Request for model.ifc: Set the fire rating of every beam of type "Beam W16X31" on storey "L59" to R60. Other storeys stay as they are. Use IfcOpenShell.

First a look at what the model holds.

```python
import ifcopenshell
import ifcopenshell.util.element

model = ifcopenshell.open("model.ifc")
print(model.schema)
storey = next(s for s in model.by_type("IfcBuildingStorey") if s.Name == "L59")
beams = [e for e in ifcopenshell.util.element.get_decomposition(storey) if e.is_a("IfcBeam")]
seen = {}
for e in beams:
    element_type = ifcopenshell.util.element.get_type(e)
    key = (element_type.Name if element_type != e and element_type else None, ifcopenshell.util.element.get_pset(e, "Pset_BeamCommon", "FireRating"))
    seen[key] = seen.get(key, 0) + 1
for (name, value), count in sorted(seen.items(), key=str):
    print(count, "x", name, "|", value)
```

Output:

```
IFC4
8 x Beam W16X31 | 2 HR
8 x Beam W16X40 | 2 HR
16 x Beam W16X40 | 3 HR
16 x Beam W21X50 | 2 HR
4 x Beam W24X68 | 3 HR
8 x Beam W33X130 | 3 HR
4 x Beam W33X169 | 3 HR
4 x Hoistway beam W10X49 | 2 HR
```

```python
import ifcopenshell
import ifcopenshell.api.pset
import ifcopenshell.util.element

model = ifcopenshell.open("model.ifc")

storey = next(s for s in model.by_type("IfcBuildingStorey") if s.Name == "L59")
beams = [e for e in ifcopenshell.util.element.get_decomposition(storey) if e.is_a("IfcBeam")]

count = 0
for e in beams:
    element_type = ifcopenshell.util.element.get_type(e)
    if element_type in (None, e) or element_type.Name != "Beam W16X31":
        continue
    found = ifcopenshell.util.element.get_pset(e, "Pset_BeamCommon", should_inherit=False)
    if found:
        pset = model.by_id(found["id"])
        if len(ifcopenshell.util.element.get_elements_by_pset(pset)) > 1:
            pset = ifcopenshell.api.pset.unshare_pset(model, products=[e], pset=pset)[0]
    else:
        pset = ifcopenshell.api.pset.add_pset(model, product=e, name="Pset_BeamCommon")
    ifcopenshell.api.pset.edit_pset(model, pset=pset, properties={"FireRating": "R60"})
    count += 1

print(count, "beams updated")

model.write("model_edited.ifc")
```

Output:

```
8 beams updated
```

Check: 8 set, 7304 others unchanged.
